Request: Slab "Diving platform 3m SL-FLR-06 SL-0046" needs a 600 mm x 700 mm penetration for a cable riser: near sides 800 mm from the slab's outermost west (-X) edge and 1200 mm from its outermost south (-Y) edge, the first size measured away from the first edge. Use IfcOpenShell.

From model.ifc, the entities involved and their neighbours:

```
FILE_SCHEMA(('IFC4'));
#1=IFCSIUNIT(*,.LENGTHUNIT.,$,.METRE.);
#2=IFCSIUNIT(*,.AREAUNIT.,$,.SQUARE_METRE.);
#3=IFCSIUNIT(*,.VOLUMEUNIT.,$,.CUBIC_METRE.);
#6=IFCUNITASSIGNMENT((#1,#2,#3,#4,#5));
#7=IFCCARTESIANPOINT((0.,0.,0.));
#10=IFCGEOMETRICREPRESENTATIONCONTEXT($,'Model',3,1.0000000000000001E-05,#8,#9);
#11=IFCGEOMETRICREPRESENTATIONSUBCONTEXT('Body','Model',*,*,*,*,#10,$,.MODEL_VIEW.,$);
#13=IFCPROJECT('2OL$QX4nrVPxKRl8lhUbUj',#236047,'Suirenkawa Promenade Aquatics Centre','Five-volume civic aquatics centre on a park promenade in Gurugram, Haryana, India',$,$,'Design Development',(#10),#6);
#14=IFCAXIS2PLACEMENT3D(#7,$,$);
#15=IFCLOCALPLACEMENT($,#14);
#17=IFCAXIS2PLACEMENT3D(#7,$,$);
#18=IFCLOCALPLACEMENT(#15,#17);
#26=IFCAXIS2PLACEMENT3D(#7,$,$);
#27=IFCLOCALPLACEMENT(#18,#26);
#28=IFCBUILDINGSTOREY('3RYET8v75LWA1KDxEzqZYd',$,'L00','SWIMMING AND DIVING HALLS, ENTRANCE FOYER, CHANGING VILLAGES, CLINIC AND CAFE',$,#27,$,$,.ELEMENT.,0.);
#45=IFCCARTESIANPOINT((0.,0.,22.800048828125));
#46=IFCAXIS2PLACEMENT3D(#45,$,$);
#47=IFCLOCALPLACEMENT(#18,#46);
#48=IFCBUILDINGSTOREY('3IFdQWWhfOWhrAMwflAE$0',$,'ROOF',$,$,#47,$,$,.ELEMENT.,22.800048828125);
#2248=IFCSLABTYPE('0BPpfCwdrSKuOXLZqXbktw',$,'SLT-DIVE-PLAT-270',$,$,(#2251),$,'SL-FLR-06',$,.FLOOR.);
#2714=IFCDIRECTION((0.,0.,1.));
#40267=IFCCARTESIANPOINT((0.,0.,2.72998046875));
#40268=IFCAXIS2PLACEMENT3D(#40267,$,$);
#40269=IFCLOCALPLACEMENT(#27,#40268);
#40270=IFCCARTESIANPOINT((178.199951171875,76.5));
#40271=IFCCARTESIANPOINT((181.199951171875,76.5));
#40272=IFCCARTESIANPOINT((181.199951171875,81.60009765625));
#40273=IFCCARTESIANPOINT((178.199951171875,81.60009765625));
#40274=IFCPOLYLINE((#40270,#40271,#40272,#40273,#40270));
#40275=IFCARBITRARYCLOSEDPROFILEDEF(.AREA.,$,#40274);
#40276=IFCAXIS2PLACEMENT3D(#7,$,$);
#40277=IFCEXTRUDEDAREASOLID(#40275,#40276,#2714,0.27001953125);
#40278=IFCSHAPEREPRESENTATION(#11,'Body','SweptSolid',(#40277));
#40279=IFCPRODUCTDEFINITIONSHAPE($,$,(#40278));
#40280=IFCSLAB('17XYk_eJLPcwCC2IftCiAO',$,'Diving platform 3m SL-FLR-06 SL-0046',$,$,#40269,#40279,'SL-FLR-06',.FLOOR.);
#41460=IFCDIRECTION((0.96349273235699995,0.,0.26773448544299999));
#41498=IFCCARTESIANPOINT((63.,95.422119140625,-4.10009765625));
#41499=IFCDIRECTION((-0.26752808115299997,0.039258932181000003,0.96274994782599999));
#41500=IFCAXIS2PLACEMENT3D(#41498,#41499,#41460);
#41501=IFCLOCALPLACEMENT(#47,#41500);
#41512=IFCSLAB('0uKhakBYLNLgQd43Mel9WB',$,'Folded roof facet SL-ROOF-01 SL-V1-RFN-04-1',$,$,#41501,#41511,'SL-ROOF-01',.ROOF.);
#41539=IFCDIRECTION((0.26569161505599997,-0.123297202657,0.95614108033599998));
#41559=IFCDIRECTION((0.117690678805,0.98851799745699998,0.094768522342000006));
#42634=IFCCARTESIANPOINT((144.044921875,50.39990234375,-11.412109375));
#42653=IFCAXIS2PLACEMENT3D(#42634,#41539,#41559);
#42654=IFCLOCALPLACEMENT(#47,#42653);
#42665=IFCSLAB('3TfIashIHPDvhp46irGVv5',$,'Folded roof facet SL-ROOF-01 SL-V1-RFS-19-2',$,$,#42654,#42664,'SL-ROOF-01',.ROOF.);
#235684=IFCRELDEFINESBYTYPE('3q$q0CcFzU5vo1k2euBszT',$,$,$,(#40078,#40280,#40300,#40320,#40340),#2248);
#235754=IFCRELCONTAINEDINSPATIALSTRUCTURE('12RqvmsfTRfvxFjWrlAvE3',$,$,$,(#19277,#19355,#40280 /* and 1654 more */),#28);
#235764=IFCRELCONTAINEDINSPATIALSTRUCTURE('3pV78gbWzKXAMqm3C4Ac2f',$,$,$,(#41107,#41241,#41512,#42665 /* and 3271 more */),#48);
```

```python
import numpy as np
import ifcopenshell
import ifcopenshell.api.feature
import ifcopenshell.api.geometry
import ifcopenshell.api.root
import ifcopenshell.geom
import ifcopenshell.util.placement
import ifcopenshell.util.representation
import ifcopenshell.util.shape
import ifcopenshell.util.unit

model = ifcopenshell.open("model.ifc")
unit_scale = ifcopenshell.util.unit.calculate_unit_scale(model)
settings = ifcopenshell.geom.settings()


def volume(element):
    """Net volume in cubic metres, openings subtracted."""
    shape = ifcopenshell.geom.create_shape(settings, element)
    return ifcopenshell.util.shape.get_volume(shape.geometry)


slab = model.by_id(40280)
before = volume(slab)

# Extent in the slab's own axes, in metres. The edges named are its -X and -Y sides.
slab_shape = ifcopenshell.geom.create_shape(settings, slab)
vertices = ifcopenshell.util.shape.get_vertices(slab_shape.geometry)
x_min, y_min, bottom = vertices.min(axis=0)
top = vertices[:, 2].max()

opening = ifcopenshell.api.root.create_entity(model, ifc_class="IfcOpeningElement", name="Cable riser opening", predefined_type="OPENING")
context = ifcopenshell.util.representation.get_context(model, "Model", "Body", "MODEL_VIEW")
width, depth = 0.6, 0.7
outline = [(0.0, 0.0), (width, 0.0), (width, depth), (0.0, depth), (0.0, 0.0)]
# Overshoot both faces by 50 mm so the cut is clean.
shape = ifcopenshell.api.geometry.add_slab_representation(
    model, context=context, depth=top - bottom + 0.1, polyline=outline
)
ifcopenshell.api.geometry.assign_representation(model, product=opening, representation=shape)

matrix = ifcopenshell.util.placement.get_local_placement(slab.ObjectPlacement)
matrix[:, 3] = matrix @ np.append(np.array([x_min + 0.8, y_min + 1.2, bottom - 0.05]) / unit_scale, 1.0)
ifcopenshell.api.geometry.edit_object_placement(model, product=opening, matrix=matrix, is_si=False)
ifcopenshell.api.feature.add_feature(model, feature=opening, element=slab)

after = volume(slab)

print(f"slab volume {before:.3f} -> {after:.3f} m3")

model.write("model_rev.ifc")
```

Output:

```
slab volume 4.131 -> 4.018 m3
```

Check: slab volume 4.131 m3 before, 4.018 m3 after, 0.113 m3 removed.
